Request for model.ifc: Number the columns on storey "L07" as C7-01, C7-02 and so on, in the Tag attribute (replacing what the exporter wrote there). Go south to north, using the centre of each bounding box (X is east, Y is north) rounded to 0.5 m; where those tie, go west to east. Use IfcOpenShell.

First a look at what the model holds.

```python
import ifcopenshell
import ifcopenshell.util.element
import ifcopenshell.util.placement

model = ifcopenshell.open("model.ifc")
print(model.schema)
storey = next(s for s in model.by_type("IfcBuildingStorey") if s.Name == "L07")
columns = [e for e in ifcopenshell.util.element.get_decomposition(storey) if e.is_a("IfcColumn")]
for e in sorted(columns, key=lambda e: e.id()):
    origin = ifcopenshell.util.placement.get_local_placement(e.ObjectPlacement)[:3, 3]
    print(e.id(), e.Tag, e.Name, origin.round(2) + 0.0, sep=" | ")
```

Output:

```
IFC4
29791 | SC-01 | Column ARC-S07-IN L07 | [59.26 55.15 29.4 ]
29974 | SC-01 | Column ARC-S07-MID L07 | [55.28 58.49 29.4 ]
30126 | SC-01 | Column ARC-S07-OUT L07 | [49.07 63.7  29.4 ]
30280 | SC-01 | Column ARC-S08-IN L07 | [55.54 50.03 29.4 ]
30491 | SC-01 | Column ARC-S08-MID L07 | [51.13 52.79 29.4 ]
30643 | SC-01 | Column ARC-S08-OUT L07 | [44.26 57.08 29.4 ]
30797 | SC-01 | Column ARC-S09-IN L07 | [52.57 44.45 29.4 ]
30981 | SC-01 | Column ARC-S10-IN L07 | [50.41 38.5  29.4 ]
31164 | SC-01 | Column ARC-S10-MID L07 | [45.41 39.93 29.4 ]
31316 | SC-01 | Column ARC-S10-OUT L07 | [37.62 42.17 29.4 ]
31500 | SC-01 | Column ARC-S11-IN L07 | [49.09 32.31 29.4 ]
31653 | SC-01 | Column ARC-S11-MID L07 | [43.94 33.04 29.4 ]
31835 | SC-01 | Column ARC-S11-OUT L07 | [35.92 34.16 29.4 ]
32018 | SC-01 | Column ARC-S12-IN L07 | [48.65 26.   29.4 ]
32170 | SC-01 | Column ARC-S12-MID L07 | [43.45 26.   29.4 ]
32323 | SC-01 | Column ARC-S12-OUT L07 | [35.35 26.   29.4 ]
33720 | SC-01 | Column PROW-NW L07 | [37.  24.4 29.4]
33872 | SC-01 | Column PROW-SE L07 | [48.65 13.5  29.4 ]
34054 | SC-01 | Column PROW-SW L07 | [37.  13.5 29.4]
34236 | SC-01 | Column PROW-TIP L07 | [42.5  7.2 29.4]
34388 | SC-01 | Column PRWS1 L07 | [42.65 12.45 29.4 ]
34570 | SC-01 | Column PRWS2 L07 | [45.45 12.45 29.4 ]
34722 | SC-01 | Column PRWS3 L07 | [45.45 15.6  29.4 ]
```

```python
import ifcopenshell
import ifcopenshell.geom
import ifcopenshell.util.element
import ifcopenshell.util.shape

model = ifcopenshell.open("model.ifc")
settings = ifcopenshell.geom.settings()
settings.set("use-world-coords", True)


def centre(element):
    shape = ifcopenshell.geom.create_shape(settings, element)
    return ifcopenshell.util.shape.get_bbox_centroid(shape.geometry)


storey = next(s for s in model.by_type("IfcBuildingStorey") if s.Name == "L07")
columns = [e for e in ifcopenshell.util.element.get_decomposition(storey) if e.is_a("IfcColumn")]

# Insertion points can sit at a corner or the storey origin, so sort by the geometry (in metres).
centres = {e: centre(e) for e in columns}
columns.sort(key=lambda e: (round(centres[e][1] / 0.5), centres[e][0]))

for i, e in enumerate(columns, start=1):
    number = f"C7-{i:02d}"
    e.Tag = number
    print(e.id(), number)

model.write("model_v2.ifc")
```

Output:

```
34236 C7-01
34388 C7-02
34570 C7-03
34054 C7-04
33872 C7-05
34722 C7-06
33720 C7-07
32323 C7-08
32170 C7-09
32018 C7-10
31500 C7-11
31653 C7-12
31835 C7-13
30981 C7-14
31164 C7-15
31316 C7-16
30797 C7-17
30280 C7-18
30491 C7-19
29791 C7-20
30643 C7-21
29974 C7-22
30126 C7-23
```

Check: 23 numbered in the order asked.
